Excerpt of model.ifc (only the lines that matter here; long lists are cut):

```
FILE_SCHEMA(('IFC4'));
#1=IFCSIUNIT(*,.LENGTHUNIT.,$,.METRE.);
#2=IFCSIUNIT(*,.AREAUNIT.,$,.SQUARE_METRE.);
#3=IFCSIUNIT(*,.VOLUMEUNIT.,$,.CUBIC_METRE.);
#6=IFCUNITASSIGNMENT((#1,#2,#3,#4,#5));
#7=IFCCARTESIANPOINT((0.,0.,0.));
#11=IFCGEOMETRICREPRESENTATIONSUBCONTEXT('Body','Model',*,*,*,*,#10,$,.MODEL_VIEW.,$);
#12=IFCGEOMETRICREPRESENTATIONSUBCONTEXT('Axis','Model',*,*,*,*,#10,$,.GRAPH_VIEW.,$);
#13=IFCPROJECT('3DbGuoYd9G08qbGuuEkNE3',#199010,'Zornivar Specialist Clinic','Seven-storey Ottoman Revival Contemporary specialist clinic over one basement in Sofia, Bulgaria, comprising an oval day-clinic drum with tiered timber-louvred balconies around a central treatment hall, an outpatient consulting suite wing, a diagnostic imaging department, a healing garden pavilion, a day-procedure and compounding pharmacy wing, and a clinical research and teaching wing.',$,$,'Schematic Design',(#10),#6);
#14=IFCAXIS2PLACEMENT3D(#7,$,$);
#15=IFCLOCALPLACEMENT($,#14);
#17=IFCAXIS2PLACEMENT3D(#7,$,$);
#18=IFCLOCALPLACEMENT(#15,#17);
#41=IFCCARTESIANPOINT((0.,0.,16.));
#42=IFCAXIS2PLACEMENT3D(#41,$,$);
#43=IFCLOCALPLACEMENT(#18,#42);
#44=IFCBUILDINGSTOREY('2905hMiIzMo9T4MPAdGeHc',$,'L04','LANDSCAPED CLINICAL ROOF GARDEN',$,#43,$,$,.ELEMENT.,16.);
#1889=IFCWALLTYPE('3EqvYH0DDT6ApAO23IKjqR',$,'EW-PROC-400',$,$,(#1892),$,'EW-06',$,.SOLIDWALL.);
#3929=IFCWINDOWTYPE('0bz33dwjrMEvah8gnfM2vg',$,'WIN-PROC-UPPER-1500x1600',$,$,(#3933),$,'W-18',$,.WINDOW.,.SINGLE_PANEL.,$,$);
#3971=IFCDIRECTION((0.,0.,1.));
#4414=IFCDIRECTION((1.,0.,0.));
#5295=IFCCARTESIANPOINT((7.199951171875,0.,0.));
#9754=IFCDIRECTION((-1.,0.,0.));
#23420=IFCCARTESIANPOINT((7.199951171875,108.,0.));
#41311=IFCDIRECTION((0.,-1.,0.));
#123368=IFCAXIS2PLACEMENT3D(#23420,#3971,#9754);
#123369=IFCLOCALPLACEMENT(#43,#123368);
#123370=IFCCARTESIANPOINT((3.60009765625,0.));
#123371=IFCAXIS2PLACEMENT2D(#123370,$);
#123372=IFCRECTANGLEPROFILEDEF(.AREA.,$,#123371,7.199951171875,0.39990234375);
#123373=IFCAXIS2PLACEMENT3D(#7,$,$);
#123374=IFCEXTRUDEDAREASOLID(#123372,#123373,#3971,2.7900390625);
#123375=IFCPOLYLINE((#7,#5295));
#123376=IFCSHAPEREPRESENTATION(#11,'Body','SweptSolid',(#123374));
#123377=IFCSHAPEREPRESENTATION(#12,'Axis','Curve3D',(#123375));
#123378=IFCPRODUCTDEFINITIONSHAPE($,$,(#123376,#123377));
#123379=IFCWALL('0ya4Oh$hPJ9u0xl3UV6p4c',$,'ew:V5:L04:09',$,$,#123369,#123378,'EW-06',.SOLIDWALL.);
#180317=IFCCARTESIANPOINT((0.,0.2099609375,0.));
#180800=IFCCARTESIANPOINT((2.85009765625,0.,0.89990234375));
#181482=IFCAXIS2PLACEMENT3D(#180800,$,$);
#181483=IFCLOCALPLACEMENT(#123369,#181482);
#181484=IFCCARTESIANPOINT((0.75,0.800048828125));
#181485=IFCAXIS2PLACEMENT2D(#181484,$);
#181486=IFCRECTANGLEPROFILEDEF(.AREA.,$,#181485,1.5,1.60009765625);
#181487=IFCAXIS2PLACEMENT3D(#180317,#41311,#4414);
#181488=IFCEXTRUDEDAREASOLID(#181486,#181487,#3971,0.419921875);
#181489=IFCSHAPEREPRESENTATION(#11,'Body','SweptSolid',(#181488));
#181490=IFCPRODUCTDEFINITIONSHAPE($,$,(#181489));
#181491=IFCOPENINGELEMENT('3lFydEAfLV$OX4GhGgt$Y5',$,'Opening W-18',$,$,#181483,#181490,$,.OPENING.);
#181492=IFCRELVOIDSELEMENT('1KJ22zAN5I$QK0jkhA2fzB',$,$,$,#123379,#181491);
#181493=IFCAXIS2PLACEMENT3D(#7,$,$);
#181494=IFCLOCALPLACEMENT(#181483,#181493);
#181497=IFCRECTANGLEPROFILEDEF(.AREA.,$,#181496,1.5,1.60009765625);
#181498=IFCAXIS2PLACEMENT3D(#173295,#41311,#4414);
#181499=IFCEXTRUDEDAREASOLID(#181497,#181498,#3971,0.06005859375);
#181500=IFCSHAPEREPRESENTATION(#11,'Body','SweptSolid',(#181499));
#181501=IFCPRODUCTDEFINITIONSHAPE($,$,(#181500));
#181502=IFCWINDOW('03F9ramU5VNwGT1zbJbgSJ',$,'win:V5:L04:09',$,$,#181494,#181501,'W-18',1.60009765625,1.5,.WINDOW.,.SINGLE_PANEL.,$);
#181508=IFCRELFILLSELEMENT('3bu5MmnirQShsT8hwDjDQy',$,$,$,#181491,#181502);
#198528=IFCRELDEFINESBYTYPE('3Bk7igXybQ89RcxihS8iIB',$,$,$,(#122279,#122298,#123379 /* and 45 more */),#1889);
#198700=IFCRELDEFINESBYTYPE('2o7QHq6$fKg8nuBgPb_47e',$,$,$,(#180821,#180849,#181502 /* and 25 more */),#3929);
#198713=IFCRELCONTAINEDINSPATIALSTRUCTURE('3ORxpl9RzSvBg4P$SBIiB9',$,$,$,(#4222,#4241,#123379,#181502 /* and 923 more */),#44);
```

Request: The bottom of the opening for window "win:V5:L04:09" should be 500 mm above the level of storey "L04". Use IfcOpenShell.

```python
import numpy as np
import ifcopenshell
import ifcopenshell.api.geometry
import ifcopenshell.geom
import ifcopenshell.util.element
import ifcopenshell.util.placement
import ifcopenshell.util.shape
import ifcopenshell.util.unit

model = ifcopenshell.open("model.ifc")
unit_scale = ifcopenshell.util.unit.calculate_unit_scale(model)

window = model.by_guid("03F9ramU5VNwGT1zbJbgSJ")
opening = window.FillsVoids[0].RelatingOpeningElement
storey = ifcopenshell.util.element.get_container(window, ifc_class="IfcBuildingStorey")
level = ifcopenshell.util.placement.get_local_placement(storey.ObjectPlacement)[2, 3]

# The opening's origin need not be at the sill, so measure its lowest point.
shape = ifcopenshell.geom.create_shape(ifcopenshell.geom.settings(), opening)
bottom = ifcopenshell.util.shape.get_shape_bottom_elevation(shape, shape.geometry) / unit_scale
dz = level + 0.5 - bottom

shift = np.array([0.0, 0.0, dz])
# The window is placed relative to its opening, so it follows when the opening moves.
matrix = ifcopenshell.util.placement.get_local_placement(opening.ObjectPlacement)
matrix[:3, 3] += shift
ifcopenshell.api.geometry.edit_object_placement(
    model, product=opening, matrix=matrix, is_si=False, should_transform_children=True
)

print(f"moved by {dz * unit_scale:+.3f} m")

model.write("model_v2.ifc")
```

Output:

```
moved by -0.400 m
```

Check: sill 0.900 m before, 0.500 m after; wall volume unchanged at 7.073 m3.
